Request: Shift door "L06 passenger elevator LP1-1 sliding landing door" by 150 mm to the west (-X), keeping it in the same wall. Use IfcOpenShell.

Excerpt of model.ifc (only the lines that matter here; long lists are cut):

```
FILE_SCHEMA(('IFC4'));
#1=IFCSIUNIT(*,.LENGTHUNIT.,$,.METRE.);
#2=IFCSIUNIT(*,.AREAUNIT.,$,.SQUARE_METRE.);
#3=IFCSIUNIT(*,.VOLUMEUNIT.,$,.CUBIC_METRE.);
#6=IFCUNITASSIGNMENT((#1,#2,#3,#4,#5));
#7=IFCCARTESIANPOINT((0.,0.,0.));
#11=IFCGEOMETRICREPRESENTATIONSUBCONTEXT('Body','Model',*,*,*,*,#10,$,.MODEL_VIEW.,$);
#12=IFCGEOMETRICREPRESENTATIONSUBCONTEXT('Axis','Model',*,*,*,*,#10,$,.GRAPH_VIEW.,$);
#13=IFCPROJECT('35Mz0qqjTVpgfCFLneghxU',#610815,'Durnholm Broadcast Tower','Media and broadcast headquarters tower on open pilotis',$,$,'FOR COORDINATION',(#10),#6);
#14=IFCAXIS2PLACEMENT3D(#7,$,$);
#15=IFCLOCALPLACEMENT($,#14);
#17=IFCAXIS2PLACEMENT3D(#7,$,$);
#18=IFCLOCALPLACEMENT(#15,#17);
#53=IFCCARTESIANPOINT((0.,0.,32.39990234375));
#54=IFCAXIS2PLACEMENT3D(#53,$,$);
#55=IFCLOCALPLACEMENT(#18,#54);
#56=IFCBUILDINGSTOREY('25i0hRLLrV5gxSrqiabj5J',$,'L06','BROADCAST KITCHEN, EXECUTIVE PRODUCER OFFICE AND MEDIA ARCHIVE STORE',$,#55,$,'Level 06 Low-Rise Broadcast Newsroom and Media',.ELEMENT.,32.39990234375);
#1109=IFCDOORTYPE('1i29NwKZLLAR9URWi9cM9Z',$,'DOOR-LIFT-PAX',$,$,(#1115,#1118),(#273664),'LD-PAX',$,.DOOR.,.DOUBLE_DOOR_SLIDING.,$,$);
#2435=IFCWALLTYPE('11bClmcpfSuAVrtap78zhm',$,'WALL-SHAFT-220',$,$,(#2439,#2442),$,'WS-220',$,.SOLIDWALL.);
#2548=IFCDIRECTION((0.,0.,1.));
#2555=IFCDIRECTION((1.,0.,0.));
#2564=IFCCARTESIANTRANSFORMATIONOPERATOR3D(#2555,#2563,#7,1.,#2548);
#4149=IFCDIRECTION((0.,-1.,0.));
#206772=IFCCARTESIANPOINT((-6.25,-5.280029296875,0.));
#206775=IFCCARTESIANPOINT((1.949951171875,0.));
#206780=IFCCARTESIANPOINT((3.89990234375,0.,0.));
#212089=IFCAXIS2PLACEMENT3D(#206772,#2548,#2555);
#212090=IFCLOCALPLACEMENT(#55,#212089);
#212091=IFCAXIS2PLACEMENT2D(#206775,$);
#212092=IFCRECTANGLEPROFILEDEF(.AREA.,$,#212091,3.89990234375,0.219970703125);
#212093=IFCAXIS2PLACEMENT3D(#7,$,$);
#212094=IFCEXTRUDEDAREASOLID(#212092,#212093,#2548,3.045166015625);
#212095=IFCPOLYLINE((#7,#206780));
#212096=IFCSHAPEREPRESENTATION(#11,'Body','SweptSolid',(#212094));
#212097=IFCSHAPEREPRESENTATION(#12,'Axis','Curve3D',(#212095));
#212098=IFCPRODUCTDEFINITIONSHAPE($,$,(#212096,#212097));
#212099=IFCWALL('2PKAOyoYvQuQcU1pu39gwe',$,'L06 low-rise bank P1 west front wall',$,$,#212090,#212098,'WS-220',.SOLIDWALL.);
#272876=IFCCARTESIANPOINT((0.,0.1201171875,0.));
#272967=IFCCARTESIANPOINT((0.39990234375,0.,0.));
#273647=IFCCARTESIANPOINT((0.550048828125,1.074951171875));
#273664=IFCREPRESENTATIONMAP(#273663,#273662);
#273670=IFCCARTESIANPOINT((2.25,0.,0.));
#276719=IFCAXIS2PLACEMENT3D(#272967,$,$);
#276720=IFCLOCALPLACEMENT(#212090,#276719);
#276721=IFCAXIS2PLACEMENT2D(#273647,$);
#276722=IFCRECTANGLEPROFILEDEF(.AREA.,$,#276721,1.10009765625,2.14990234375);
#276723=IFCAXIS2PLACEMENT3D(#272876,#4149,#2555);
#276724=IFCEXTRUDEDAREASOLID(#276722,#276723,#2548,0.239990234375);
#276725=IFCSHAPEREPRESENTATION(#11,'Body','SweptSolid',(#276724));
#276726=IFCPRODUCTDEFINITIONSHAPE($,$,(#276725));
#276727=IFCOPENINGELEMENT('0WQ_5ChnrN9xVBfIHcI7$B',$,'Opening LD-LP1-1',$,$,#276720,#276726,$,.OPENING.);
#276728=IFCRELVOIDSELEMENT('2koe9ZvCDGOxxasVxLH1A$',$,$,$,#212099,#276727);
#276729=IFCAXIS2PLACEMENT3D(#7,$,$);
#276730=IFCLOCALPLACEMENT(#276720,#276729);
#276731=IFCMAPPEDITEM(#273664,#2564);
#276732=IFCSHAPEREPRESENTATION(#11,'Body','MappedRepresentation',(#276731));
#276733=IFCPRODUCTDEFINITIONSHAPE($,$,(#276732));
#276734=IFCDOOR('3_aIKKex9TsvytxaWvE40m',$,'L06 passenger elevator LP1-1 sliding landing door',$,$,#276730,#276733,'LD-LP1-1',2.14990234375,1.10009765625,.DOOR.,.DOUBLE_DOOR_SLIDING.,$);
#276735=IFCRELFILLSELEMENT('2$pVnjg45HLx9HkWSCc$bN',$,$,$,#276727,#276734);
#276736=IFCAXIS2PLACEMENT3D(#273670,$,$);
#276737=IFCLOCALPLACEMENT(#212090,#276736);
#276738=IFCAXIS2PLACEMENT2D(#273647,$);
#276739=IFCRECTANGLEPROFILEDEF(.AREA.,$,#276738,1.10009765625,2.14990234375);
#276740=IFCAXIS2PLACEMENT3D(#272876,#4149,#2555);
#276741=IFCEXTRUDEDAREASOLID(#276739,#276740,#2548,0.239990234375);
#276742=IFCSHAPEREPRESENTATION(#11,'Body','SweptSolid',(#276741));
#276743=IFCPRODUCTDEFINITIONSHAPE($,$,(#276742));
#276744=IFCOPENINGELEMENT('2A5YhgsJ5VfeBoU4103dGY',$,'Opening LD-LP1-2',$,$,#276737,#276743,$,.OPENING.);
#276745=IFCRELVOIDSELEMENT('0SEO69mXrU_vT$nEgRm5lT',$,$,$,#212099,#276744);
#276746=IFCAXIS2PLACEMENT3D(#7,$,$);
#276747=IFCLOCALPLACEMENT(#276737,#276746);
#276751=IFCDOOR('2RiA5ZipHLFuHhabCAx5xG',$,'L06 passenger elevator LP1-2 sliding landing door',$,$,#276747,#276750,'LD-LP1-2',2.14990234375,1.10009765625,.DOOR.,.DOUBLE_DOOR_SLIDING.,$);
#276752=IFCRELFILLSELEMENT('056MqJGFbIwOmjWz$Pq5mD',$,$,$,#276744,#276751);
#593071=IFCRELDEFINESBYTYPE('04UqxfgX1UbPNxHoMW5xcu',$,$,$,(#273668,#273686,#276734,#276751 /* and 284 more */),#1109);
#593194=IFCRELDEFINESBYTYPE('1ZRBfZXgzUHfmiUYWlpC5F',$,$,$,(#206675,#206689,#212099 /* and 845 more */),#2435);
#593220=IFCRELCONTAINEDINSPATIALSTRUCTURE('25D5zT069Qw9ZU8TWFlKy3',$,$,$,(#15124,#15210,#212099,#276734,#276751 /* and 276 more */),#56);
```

```python
import ifcopenshell
import ifcopenshell.api.geometry
import ifcopenshell.util.placement
import ifcopenshell.util.unit

model = ifcopenshell.open("model.ifc")
unit_scale = ifcopenshell.util.unit.calculate_unit_scale(model)

door = model.by_guid("3_aIKKex9TsvytxaWvE40m")
opening = door.FillsVoids[0].RelatingOpeningElement
wall = opening.VoidsElements[0].RelatingBuildingElement

wall_matrix = ifcopenshell.util.placement.get_local_placement(wall.ObjectPlacement)
shift = wall_matrix[:3, 0] * -0.15 / unit_scale
before = ifcopenshell.util.placement.get_local_placement(door.ObjectPlacement)[:3, 3].copy()

# The door is placed relative to its opening, so it follows when the opening moves.
matrix = ifcopenshell.util.placement.get_local_placement(opening.ObjectPlacement)
matrix[:3, 3] += shift
ifcopenshell.api.geometry.edit_object_placement(
    model, product=opening, matrix=matrix, is_si=False, should_transform_children=True
)

after = ifcopenshell.util.placement.get_local_placement(door.ObjectPlacement)[:3, 3]
print("door moved by", (after - before).round(3) + 0.0)

model.write("model_updated.ifc")
```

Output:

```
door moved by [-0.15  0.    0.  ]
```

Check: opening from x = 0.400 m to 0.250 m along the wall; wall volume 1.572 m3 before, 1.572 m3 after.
